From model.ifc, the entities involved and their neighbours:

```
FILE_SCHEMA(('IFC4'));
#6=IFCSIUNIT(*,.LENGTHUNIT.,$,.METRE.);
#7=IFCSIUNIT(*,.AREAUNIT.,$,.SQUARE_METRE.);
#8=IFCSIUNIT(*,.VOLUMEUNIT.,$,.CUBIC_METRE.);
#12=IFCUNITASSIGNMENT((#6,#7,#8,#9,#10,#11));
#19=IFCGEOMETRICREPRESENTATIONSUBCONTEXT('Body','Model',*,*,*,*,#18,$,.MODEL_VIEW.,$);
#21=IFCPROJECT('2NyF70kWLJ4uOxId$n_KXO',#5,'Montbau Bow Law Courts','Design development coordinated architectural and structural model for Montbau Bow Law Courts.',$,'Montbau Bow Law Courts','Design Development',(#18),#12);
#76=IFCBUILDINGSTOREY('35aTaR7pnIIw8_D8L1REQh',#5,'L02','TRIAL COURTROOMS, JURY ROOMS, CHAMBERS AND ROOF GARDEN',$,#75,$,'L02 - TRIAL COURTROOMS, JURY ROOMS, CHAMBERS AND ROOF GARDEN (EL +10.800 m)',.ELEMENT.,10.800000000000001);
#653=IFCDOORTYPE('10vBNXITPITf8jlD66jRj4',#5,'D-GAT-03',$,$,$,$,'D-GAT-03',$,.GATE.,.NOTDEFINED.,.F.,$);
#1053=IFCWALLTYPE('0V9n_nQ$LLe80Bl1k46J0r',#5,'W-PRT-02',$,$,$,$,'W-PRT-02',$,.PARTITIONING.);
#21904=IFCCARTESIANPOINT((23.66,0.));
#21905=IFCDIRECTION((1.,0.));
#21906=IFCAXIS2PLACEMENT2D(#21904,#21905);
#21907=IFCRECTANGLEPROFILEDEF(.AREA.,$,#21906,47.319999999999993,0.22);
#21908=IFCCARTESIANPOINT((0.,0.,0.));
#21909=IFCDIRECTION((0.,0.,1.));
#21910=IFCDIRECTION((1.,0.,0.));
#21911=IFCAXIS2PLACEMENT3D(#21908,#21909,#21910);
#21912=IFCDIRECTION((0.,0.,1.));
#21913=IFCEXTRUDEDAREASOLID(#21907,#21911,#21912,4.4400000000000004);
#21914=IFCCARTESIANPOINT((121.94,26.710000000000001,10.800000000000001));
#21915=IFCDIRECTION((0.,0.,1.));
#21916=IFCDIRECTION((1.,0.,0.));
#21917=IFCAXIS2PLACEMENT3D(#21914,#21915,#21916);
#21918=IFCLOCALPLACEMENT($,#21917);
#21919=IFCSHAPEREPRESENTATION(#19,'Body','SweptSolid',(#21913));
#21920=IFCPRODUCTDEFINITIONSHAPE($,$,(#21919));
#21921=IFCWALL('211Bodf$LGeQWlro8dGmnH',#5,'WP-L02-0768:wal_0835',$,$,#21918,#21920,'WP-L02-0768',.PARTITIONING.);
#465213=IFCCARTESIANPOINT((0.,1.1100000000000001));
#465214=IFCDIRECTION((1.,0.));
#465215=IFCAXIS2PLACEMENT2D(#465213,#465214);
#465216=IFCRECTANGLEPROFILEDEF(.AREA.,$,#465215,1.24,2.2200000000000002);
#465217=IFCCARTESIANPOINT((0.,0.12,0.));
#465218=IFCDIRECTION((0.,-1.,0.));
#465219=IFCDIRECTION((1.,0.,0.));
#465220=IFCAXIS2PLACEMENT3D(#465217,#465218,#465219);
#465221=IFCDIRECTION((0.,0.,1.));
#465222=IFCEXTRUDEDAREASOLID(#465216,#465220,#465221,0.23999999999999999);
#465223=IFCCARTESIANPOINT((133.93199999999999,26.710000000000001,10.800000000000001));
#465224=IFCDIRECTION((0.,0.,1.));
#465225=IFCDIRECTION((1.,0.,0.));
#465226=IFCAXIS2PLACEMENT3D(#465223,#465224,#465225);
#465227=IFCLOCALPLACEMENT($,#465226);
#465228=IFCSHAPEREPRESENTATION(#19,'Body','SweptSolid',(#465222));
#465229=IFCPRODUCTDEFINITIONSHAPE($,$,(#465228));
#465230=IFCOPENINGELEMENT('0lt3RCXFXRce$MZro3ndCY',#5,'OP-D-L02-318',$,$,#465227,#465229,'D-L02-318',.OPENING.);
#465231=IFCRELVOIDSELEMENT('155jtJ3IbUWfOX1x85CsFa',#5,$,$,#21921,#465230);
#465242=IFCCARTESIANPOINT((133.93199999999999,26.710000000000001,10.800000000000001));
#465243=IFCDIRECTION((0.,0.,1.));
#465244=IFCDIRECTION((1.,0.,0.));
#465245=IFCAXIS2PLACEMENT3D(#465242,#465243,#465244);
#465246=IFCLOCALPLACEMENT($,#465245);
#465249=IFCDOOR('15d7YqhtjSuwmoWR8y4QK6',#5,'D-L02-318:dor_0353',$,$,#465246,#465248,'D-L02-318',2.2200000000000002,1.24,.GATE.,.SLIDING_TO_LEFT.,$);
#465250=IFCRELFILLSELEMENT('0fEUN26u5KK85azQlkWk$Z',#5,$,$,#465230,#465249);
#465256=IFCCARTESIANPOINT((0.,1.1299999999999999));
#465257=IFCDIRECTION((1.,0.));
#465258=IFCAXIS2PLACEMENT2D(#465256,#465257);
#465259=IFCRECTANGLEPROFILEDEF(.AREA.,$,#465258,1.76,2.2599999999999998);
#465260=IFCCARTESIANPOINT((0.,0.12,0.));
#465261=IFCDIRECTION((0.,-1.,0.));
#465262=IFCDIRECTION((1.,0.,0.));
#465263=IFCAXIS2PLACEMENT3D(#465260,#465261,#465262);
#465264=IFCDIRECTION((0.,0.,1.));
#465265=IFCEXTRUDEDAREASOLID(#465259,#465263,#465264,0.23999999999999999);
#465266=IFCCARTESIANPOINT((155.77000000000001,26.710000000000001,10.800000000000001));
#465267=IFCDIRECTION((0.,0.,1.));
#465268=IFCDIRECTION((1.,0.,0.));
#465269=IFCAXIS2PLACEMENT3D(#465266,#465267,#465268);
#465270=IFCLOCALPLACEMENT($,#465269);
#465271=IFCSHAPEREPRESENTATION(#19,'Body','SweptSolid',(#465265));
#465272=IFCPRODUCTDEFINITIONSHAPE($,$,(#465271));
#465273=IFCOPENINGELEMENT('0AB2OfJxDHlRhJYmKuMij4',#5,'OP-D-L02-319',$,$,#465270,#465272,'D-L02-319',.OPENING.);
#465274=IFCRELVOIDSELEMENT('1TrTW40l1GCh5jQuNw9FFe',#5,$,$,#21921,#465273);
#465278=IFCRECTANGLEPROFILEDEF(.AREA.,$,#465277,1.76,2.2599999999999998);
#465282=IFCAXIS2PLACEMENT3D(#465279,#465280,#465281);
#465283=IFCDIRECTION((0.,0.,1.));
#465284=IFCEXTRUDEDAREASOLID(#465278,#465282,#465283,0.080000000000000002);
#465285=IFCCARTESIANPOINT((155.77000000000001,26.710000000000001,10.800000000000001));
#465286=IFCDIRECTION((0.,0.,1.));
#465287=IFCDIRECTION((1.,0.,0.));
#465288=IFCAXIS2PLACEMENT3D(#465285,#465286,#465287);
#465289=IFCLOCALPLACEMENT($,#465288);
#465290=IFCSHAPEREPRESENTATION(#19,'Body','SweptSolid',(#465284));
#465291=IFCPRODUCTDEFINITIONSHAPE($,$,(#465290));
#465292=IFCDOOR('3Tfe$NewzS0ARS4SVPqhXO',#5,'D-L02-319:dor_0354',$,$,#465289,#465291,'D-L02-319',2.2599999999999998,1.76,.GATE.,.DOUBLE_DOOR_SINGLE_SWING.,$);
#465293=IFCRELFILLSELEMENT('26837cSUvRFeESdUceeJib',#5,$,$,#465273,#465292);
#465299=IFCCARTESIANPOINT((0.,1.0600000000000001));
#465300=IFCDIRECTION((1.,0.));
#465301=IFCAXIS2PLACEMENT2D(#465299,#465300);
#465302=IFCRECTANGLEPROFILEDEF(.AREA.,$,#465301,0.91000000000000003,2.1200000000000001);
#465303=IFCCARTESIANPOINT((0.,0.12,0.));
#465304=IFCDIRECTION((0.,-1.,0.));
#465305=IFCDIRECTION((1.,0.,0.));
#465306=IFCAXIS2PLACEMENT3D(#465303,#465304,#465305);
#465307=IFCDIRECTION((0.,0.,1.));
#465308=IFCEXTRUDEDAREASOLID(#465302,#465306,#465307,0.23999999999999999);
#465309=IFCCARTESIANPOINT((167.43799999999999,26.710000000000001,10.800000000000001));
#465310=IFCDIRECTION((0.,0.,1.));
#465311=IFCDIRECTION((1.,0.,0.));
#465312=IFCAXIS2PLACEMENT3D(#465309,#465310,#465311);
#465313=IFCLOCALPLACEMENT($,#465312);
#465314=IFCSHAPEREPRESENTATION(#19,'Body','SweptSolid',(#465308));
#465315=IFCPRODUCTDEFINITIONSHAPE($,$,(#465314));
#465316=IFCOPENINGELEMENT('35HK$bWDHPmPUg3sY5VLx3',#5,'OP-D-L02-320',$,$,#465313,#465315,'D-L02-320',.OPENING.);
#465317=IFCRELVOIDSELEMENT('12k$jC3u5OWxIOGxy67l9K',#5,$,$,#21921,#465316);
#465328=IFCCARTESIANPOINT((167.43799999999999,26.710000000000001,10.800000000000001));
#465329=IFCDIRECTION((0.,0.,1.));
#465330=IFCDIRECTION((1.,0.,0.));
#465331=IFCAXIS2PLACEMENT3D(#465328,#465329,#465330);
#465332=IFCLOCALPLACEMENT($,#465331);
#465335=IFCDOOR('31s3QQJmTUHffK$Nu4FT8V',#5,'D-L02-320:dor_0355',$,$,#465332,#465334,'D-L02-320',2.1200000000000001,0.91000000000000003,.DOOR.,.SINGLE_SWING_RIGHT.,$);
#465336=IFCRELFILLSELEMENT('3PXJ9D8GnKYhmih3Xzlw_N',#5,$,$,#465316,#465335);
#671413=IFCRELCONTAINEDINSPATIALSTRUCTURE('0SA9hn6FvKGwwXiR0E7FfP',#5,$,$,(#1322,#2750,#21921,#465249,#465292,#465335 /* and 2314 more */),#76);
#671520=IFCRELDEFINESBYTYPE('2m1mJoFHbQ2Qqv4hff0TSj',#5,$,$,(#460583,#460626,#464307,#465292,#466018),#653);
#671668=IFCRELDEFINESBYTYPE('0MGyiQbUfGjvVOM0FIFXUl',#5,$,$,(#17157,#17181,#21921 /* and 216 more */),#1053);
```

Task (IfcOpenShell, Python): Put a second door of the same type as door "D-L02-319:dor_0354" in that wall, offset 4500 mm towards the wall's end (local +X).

```python
import ifcopenshell
import ifcopenshell.api.feature
import ifcopenshell.api.geometry
import ifcopenshell.api.root
import ifcopenshell.geom
import ifcopenshell.util.element
import ifcopenshell.util.placement
import ifcopenshell.util.shape

model = ifcopenshell.open("model.ifc")
settings = ifcopenshell.geom.settings()


def volume(element):
    """Net volume in cubic metres, openings subtracted."""
    shape = ifcopenshell.geom.create_shape(settings, element)
    return ifcopenshell.util.shape.get_volume(shape.geometry)


def reuse_history(source, copy):
    """copy_class also copies each property set's owner history, people and application; keep the originals."""
    for rel in copy.IsDefinedBy:
        if rel.is_a("IfcRelDefinesByProperties") and (history := rel.RelatingPropertyDefinition.OwnerHistory):
            rel.RelatingPropertyDefinition.OwnerHistory = source.OwnerHistory
            ifcopenshell.util.element.remove_deep2(model, history)


door = model.by_id(465292)
opening = door.FillsVoids[0].RelatingOpeningElement
wall = opening.VoidsElements[0].RelatingBuildingElement
before = volume(wall)
shift = ifcopenshell.util.placement.get_local_placement(wall.ObjectPlacement)[:3, 0] * 4.5

# copy_class copies the void relationship, type, container and properties, but no geometry.
new_opening = ifcopenshell.api.root.copy_class(model, product=opening)
new_opening.Representation = ifcopenshell.util.element.copy_deep(
    model, opening.Representation, exclude=["IfcGeometricRepresentationContext", "IfcRepresentationMap"]
)
new_opening.Tag = None
new_door = ifcopenshell.api.root.copy_class(model, product=door)
new_door.Representation = ifcopenshell.util.element.copy_deep(
    model, door.Representation, exclude=["IfcGeometricRepresentationContext", "IfcRepresentationMap"]
)
new_door.Tag = None
reuse_history(door, new_door)
ifcopenshell.api.feature.add_filling(model, opening=new_opening, element=new_door)

for old, new in ((opening, new_opening), (door, new_door)):
    matrix = ifcopenshell.util.placement.get_local_placement(old.ObjectPlacement)
    matrix[:3, 3] += shift
    ifcopenshell.api.geometry.edit_object_placement(model, product=new, matrix=matrix, is_si=False)

after = volume(wall)

print(f"wall volume {before:.3f} -> {after:.3f} m3")

model.write("model_v2.ifc")
```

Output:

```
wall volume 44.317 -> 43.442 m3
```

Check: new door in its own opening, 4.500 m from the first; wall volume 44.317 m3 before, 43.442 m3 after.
